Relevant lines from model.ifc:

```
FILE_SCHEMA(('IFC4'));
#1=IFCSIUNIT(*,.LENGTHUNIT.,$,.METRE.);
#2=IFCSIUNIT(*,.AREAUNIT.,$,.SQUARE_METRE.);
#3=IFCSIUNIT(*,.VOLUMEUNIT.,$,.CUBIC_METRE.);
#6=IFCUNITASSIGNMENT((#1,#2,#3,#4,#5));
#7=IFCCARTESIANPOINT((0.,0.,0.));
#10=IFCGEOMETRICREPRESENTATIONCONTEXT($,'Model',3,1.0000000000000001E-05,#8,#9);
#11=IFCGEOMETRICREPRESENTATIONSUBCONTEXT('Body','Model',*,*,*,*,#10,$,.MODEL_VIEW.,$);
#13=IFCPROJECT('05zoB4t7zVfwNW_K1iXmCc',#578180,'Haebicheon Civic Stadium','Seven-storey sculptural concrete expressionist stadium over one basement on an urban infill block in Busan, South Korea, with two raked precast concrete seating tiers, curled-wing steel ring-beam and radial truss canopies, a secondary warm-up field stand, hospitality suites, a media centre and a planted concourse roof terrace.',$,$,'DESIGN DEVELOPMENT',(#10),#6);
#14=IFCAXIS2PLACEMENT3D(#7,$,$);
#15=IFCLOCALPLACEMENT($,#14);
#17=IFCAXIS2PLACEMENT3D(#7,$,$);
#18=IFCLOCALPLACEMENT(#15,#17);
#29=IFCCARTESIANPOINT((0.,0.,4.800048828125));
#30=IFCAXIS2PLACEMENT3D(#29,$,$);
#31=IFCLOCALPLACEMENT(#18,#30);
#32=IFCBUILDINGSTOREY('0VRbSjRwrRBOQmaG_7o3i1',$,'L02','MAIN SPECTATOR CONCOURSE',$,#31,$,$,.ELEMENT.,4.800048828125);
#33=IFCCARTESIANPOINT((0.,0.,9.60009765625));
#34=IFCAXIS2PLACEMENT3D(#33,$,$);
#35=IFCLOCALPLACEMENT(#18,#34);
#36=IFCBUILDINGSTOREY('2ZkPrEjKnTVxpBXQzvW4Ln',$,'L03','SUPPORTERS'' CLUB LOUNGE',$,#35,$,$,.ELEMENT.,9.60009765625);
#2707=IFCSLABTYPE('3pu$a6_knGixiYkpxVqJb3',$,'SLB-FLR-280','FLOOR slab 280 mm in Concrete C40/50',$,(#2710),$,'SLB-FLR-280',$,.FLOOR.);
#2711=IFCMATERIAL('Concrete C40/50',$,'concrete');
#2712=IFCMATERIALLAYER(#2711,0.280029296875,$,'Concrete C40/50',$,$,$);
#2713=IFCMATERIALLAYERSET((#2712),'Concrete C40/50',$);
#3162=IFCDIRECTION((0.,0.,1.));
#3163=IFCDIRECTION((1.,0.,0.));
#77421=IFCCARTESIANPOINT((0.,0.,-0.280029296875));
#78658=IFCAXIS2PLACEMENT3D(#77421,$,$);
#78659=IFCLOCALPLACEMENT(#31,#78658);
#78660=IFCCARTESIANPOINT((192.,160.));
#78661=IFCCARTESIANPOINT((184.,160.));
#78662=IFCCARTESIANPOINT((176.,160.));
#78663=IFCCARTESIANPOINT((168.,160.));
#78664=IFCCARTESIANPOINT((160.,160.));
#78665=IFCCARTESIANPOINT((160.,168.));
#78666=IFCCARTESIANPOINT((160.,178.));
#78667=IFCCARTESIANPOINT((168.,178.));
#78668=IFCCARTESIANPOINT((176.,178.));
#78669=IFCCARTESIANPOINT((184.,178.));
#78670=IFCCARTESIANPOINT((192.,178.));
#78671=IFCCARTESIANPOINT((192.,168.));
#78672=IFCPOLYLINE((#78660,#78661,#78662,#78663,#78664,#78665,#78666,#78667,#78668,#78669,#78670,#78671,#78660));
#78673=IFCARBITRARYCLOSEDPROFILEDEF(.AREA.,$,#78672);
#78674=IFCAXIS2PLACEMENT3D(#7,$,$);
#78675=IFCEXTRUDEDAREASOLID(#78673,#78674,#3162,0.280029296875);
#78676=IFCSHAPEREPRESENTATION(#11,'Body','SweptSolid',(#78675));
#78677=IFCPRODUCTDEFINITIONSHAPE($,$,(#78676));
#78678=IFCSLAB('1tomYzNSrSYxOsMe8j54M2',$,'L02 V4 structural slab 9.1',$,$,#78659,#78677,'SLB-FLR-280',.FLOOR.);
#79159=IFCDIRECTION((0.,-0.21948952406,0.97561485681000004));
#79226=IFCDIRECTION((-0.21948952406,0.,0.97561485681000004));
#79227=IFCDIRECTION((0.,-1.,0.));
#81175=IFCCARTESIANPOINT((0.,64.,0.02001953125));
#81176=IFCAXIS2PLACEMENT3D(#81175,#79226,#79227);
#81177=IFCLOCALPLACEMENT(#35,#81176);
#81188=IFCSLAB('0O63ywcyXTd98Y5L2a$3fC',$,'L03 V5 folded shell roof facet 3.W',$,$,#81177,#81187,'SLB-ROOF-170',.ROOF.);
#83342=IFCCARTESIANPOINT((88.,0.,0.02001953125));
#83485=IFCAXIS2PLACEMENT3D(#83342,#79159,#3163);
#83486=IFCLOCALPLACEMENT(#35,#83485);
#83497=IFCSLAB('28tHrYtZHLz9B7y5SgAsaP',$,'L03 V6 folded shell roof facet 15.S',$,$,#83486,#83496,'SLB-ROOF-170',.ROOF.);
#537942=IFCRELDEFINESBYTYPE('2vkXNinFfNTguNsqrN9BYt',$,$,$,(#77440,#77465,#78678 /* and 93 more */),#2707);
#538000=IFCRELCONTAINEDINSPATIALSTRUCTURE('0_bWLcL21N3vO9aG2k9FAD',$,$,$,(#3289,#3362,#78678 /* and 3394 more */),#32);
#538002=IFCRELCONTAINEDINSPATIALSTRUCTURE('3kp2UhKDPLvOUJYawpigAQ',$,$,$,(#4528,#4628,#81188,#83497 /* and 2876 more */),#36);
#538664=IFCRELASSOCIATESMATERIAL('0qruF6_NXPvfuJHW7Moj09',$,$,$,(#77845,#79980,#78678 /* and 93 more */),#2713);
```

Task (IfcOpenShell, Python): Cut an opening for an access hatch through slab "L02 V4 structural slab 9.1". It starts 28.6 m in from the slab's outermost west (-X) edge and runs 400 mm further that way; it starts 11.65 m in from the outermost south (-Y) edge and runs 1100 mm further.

```python
import numpy as np
import ifcopenshell
import ifcopenshell.api.feature
import ifcopenshell.api.geometry
import ifcopenshell.api.root
import ifcopenshell.geom
import ifcopenshell.util.placement
import ifcopenshell.util.representation
import ifcopenshell.util.shape
import ifcopenshell.util.unit

model = ifcopenshell.open("model.ifc")
unit_scale = ifcopenshell.util.unit.calculate_unit_scale(model)
settings = ifcopenshell.geom.settings()


def volume(element):
    """Net volume in cubic metres, openings subtracted."""
    shape = ifcopenshell.geom.create_shape(settings, element)
    return ifcopenshell.util.shape.get_volume(shape.geometry)


slab = model.by_guid("1tomYzNSrSYxOsMe8j54M2")
before = volume(slab)

# Extent in the slab's own axes, in metres. The edges named are its -X and -Y sides.
slab_shape = ifcopenshell.geom.create_shape(settings, slab)
vertices = ifcopenshell.util.shape.get_vertices(slab_shape.geometry)
x_min, y_min, bottom = vertices.min(axis=0)
top = vertices[:, 2].max()

opening = ifcopenshell.api.root.create_entity(model, ifc_class="IfcOpeningElement", name="Access hatch opening", predefined_type="OPENING")
context = ifcopenshell.util.representation.get_context(model, "Model", "Body", "MODEL_VIEW")
width, depth = 0.4, 1.1
outline = [(0.0, 0.0), (width, 0.0), (width, depth), (0.0, depth), (0.0, 0.0)]
# Overshoot both faces by 50 mm so the cut is clean.
shape = ifcopenshell.api.geometry.add_slab_representation(
    model, context=context, depth=top - bottom + 0.1, polyline=outline
)
ifcopenshell.api.geometry.assign_representation(model, product=opening, representation=shape)

matrix = ifcopenshell.util.placement.get_local_placement(slab.ObjectPlacement)
matrix[:, 3] = matrix @ np.append(np.array([x_min + 28.6, y_min + 11.65, bottom - 0.05]) / unit_scale, 1.0)
ifcopenshell.api.geometry.edit_object_placement(model, product=opening, matrix=matrix, is_si=False)
ifcopenshell.api.feature.add_feature(model, feature=opening, element=slab)

after = volume(slab)

print(f"slab volume {before:.3f} -> {after:.3f} m3")

model.write("model-out.ifc")
```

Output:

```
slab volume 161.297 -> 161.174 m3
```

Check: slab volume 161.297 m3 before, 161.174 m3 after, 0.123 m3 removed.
